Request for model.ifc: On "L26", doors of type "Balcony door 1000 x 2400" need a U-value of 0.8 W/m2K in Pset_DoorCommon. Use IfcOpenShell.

First a look at what the model holds.

```python
import ifcopenshell
import ifcopenshell.util.element

model = ifcopenshell.open("model.ifc")
print(model.schema)
storey = next(s for s in model.by_type("IfcBuildingStorey") if s.Name == "L26")
doors = [e for e in ifcopenshell.util.element.get_decomposition(storey) if e.is_a("IfcDoor")]
seen = {}
for e in doors:
    element_type = ifcopenshell.util.element.get_type(e)
    key = (element_type.Name if element_type != e and element_type else None, ifcopenshell.util.element.get_pset(e, "Pset_DoorCommon", "ThermalTransmittance"))
    seen[key] = seen.get(key, 0) + 1
for (name, value), count in sorted(seen.items(), key=str):
    print(count, "x", name, "|", value)
```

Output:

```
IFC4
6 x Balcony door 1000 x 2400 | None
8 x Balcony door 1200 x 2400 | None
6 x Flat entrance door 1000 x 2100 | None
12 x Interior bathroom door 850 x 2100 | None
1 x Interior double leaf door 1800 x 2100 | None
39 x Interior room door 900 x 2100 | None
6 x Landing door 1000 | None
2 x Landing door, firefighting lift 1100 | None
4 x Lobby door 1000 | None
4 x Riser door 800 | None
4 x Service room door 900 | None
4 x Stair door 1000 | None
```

```python
import ifcopenshell
import ifcopenshell.api.pset
import ifcopenshell.util.element

model = ifcopenshell.open("model.ifc")

storey = next(s for s in model.by_type("IfcBuildingStorey") if s.Name == "L26")
doors = [e for e in ifcopenshell.util.element.get_decomposition(storey) if e.is_a("IfcDoor")]

count = 0
for e in doors:
    element_type = ifcopenshell.util.element.get_type(e)
    if element_type in (None, e) or element_type.Name != "Balcony door 1000 x 2400":
        continue
    # add_pset returns the element's existing set when there is one.
    pset = ifcopenshell.api.pset.add_pset(model, product=e, name="Pset_DoorCommon")
    ifcopenshell.api.pset.edit_pset(model, pset=pset, properties={"ThermalTransmittance": 0.8})
    count += 1

print(count, "doors updated")

model.write("model_rev.ifc")
```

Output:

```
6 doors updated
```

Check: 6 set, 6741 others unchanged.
